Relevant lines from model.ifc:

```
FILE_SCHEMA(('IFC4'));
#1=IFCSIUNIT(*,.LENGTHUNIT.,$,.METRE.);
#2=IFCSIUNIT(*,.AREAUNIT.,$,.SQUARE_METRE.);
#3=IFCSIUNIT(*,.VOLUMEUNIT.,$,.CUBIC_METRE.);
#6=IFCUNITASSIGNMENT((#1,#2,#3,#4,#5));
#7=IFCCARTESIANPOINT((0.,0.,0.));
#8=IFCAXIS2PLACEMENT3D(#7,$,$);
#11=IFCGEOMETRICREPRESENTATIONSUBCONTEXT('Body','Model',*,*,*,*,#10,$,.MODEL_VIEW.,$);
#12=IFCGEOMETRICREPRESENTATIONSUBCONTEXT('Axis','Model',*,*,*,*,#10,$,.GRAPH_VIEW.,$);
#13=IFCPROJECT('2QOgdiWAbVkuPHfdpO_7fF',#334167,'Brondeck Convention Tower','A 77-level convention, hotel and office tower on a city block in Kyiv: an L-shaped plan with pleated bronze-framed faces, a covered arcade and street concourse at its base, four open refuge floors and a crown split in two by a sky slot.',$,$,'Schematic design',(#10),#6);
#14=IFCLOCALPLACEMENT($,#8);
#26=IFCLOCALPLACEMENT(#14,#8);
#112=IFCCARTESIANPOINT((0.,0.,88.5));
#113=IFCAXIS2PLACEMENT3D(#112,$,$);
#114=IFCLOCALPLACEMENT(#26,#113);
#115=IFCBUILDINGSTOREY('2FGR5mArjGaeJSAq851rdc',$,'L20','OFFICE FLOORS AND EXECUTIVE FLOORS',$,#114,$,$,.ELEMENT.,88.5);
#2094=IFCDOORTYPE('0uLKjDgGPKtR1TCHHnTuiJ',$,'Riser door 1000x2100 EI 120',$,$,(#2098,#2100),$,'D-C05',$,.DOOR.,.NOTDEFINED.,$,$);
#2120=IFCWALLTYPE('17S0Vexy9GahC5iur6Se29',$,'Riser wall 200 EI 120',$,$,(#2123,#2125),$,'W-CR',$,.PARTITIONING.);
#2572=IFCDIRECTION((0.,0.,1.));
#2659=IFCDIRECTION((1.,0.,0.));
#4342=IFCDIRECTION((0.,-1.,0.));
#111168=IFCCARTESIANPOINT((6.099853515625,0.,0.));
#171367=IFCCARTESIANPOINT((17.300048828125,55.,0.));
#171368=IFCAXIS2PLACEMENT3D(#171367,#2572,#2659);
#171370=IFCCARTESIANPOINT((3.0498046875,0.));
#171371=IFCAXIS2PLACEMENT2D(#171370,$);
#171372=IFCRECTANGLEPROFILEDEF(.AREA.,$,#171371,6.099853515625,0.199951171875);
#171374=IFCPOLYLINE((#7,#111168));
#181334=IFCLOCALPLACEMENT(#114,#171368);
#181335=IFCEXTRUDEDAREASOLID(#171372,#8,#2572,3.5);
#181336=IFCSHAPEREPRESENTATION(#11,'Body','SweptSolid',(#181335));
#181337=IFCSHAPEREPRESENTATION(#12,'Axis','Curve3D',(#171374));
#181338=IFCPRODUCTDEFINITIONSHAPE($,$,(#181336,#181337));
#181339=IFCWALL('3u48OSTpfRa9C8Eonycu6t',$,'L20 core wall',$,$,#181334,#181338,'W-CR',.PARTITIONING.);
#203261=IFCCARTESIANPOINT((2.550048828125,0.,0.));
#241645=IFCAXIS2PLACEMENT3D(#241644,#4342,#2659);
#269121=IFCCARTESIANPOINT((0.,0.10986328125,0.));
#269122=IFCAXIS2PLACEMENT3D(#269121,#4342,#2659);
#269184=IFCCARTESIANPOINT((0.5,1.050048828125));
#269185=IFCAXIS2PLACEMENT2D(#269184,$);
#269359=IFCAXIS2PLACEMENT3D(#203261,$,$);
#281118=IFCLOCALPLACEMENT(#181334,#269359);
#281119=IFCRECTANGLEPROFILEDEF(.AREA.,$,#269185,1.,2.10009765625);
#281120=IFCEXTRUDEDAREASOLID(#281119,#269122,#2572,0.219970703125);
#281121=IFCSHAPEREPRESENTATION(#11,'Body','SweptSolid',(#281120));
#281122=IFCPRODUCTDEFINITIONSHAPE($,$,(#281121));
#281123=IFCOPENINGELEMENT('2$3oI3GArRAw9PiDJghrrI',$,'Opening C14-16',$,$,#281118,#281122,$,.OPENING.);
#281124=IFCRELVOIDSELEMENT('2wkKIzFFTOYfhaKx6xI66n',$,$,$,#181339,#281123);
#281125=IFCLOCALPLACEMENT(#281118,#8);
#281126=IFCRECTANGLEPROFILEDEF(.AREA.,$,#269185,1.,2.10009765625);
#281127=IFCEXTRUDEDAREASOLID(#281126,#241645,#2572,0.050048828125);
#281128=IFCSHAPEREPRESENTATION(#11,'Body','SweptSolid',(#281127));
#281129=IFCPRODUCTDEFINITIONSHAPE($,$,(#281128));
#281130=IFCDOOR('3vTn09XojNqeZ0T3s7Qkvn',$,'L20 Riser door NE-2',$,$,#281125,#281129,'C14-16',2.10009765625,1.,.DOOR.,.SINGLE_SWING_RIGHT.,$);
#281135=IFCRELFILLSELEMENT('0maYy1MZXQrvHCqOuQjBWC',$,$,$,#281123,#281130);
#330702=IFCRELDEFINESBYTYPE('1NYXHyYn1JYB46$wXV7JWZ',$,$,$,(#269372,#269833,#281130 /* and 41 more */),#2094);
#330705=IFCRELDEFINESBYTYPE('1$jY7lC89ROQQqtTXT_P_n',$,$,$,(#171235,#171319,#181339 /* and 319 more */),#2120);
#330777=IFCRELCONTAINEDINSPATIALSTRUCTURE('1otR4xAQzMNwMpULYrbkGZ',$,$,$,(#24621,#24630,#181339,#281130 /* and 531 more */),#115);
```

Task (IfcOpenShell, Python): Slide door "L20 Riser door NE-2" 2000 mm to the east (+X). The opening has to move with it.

```python
import ifcopenshell
import ifcopenshell.api.geometry
import ifcopenshell.util.placement

model = ifcopenshell.open("model.ifc")

door = model.by_id(281130)
opening = door.FillsVoids[0].RelatingOpeningElement
wall = opening.VoidsElements[0].RelatingBuildingElement

wall_matrix = ifcopenshell.util.placement.get_local_placement(wall.ObjectPlacement)
shift = wall_matrix[:3, 0] * 2.0
before = ifcopenshell.util.placement.get_local_placement(door.ObjectPlacement)[:3, 3].copy()

# The door is placed relative to its opening, so it follows when the opening moves.
matrix = ifcopenshell.util.placement.get_local_placement(opening.ObjectPlacement)
matrix[:3, 3] += shift
ifcopenshell.api.geometry.edit_object_placement(
    model, product=opening, matrix=matrix, is_si=False, should_transform_children=True
)

after = ifcopenshell.util.placement.get_local_placement(door.ObjectPlacement)[:3, 3]
print("door moved by", (after - before).round(3) + 0.0)

model.write("model_updated.ifc")
```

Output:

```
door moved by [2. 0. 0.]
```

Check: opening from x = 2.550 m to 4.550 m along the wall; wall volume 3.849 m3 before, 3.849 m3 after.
